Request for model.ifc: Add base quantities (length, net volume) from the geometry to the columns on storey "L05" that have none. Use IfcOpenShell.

First a look at what the model holds.

```python
import ifcopenshell
import ifcopenshell.util.element
import ifcopenshell.util.unit

model = ifcopenshell.open("model.ifc")
print(model.schema)
for unit_type in ("LENGTHUNIT", "AREAUNIT", "VOLUMEUNIT"):
    print(unit_type, ifcopenshell.util.unit.calculate_unit_scale(model, unit_type))
storey = next(s for s in model.by_type("IfcBuildingStorey") if s.Name == "L05")
columns = [e for e in ifcopenshell.util.element.get_decomposition(storey) if e.is_a("IfcColumn")]
for e in sorted(columns, key=lambda e: e.id()):
    print(e.id(), e.is_a(), e.Name, list(ifcopenshell.util.element.get_psets(e, qtos_only=True)), sep=" | ")
```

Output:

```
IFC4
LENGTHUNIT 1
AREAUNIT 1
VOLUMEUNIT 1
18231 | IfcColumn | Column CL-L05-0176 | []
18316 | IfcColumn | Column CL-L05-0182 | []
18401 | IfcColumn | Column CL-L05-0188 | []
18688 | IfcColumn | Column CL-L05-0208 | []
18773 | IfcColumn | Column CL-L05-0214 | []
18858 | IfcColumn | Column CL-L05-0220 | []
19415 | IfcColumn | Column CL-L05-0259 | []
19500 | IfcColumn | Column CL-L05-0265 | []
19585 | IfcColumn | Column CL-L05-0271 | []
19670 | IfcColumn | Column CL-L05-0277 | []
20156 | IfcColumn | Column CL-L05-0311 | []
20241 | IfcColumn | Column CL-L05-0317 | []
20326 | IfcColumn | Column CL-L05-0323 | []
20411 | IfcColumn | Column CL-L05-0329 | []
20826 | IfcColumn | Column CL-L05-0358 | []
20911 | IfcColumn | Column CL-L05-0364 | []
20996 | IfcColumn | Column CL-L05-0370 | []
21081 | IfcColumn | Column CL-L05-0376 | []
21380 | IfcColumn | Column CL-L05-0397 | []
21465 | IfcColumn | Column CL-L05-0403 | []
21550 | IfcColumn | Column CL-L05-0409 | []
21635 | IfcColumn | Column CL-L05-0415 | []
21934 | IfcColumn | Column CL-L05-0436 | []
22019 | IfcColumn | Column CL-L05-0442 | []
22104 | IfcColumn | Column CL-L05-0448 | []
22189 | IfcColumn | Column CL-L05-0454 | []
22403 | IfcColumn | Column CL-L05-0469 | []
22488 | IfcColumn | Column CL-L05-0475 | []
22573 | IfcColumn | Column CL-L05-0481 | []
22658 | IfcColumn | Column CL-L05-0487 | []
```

```python
import ifcopenshell
import ifcopenshell.api.pset
import ifcopenshell.geom
import ifcopenshell.util.element
import ifcopenshell.util.shape
import ifcopenshell.util.unit

model = ifcopenshell.open("model.ifc")
unit_scale = ifcopenshell.util.unit.calculate_unit_scale(model)
volume_scale = ifcopenshell.util.unit.calculate_unit_scale(model, "VOLUMEUNIT")
settings = ifcopenshell.geom.settings()

storey = next(s for s in model.by_type("IfcBuildingStorey") if s.Name == "L05")
columns = [e for e in ifcopenshell.util.element.get_decomposition(storey) if e.is_a("IfcColumn")]

for e in sorted(columns, key=lambda e: e.id()):
    if ifcopenshell.util.element.get_psets(e, qtos_only=True, should_inherit=False):
        continue
    # Geometry comes back in metres, in the element's own axes.
    shape = ifcopenshell.geom.create_shape(settings, e)
    values = {
        "Length": ifcopenshell.util.shape.get_z(shape.geometry) / unit_scale,
        "NetVolume": ifcopenshell.util.shape.get_volume(shape.geometry) / volume_scale,
    }
    qto = ifcopenshell.api.pset.add_qto(model, product=e, name="Qto_ColumnBaseQuantities")
    ifcopenshell.api.pset.edit_qto(model, qto=qto, properties=values)
    print(e.id(), {k: round(v, 3) for k, v in values.items()})

model.write("model-out.ifc")
```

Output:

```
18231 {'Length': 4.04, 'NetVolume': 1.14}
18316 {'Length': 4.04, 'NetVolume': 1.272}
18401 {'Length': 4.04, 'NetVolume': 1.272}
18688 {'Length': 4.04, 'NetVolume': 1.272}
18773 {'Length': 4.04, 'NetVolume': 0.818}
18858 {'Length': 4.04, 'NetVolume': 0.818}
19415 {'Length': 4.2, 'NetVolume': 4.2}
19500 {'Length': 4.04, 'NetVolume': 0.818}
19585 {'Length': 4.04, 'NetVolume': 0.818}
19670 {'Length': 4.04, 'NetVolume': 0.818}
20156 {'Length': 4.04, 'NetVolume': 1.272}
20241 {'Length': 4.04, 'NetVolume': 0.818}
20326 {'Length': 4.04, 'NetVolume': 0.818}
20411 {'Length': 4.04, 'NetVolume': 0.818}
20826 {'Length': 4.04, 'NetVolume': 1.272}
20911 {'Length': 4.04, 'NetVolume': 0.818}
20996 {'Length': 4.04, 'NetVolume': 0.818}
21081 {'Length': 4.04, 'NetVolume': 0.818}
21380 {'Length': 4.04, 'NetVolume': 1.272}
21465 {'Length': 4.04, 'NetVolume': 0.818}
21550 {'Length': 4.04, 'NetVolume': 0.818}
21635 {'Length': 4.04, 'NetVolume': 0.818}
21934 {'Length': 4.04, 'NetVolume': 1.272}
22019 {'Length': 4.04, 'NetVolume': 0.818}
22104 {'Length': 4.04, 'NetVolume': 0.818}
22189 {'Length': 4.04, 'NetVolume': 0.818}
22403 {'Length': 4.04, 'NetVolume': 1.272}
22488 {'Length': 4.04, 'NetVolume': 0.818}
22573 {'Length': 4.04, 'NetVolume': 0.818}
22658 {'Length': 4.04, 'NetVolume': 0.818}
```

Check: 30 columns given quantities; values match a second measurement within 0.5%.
